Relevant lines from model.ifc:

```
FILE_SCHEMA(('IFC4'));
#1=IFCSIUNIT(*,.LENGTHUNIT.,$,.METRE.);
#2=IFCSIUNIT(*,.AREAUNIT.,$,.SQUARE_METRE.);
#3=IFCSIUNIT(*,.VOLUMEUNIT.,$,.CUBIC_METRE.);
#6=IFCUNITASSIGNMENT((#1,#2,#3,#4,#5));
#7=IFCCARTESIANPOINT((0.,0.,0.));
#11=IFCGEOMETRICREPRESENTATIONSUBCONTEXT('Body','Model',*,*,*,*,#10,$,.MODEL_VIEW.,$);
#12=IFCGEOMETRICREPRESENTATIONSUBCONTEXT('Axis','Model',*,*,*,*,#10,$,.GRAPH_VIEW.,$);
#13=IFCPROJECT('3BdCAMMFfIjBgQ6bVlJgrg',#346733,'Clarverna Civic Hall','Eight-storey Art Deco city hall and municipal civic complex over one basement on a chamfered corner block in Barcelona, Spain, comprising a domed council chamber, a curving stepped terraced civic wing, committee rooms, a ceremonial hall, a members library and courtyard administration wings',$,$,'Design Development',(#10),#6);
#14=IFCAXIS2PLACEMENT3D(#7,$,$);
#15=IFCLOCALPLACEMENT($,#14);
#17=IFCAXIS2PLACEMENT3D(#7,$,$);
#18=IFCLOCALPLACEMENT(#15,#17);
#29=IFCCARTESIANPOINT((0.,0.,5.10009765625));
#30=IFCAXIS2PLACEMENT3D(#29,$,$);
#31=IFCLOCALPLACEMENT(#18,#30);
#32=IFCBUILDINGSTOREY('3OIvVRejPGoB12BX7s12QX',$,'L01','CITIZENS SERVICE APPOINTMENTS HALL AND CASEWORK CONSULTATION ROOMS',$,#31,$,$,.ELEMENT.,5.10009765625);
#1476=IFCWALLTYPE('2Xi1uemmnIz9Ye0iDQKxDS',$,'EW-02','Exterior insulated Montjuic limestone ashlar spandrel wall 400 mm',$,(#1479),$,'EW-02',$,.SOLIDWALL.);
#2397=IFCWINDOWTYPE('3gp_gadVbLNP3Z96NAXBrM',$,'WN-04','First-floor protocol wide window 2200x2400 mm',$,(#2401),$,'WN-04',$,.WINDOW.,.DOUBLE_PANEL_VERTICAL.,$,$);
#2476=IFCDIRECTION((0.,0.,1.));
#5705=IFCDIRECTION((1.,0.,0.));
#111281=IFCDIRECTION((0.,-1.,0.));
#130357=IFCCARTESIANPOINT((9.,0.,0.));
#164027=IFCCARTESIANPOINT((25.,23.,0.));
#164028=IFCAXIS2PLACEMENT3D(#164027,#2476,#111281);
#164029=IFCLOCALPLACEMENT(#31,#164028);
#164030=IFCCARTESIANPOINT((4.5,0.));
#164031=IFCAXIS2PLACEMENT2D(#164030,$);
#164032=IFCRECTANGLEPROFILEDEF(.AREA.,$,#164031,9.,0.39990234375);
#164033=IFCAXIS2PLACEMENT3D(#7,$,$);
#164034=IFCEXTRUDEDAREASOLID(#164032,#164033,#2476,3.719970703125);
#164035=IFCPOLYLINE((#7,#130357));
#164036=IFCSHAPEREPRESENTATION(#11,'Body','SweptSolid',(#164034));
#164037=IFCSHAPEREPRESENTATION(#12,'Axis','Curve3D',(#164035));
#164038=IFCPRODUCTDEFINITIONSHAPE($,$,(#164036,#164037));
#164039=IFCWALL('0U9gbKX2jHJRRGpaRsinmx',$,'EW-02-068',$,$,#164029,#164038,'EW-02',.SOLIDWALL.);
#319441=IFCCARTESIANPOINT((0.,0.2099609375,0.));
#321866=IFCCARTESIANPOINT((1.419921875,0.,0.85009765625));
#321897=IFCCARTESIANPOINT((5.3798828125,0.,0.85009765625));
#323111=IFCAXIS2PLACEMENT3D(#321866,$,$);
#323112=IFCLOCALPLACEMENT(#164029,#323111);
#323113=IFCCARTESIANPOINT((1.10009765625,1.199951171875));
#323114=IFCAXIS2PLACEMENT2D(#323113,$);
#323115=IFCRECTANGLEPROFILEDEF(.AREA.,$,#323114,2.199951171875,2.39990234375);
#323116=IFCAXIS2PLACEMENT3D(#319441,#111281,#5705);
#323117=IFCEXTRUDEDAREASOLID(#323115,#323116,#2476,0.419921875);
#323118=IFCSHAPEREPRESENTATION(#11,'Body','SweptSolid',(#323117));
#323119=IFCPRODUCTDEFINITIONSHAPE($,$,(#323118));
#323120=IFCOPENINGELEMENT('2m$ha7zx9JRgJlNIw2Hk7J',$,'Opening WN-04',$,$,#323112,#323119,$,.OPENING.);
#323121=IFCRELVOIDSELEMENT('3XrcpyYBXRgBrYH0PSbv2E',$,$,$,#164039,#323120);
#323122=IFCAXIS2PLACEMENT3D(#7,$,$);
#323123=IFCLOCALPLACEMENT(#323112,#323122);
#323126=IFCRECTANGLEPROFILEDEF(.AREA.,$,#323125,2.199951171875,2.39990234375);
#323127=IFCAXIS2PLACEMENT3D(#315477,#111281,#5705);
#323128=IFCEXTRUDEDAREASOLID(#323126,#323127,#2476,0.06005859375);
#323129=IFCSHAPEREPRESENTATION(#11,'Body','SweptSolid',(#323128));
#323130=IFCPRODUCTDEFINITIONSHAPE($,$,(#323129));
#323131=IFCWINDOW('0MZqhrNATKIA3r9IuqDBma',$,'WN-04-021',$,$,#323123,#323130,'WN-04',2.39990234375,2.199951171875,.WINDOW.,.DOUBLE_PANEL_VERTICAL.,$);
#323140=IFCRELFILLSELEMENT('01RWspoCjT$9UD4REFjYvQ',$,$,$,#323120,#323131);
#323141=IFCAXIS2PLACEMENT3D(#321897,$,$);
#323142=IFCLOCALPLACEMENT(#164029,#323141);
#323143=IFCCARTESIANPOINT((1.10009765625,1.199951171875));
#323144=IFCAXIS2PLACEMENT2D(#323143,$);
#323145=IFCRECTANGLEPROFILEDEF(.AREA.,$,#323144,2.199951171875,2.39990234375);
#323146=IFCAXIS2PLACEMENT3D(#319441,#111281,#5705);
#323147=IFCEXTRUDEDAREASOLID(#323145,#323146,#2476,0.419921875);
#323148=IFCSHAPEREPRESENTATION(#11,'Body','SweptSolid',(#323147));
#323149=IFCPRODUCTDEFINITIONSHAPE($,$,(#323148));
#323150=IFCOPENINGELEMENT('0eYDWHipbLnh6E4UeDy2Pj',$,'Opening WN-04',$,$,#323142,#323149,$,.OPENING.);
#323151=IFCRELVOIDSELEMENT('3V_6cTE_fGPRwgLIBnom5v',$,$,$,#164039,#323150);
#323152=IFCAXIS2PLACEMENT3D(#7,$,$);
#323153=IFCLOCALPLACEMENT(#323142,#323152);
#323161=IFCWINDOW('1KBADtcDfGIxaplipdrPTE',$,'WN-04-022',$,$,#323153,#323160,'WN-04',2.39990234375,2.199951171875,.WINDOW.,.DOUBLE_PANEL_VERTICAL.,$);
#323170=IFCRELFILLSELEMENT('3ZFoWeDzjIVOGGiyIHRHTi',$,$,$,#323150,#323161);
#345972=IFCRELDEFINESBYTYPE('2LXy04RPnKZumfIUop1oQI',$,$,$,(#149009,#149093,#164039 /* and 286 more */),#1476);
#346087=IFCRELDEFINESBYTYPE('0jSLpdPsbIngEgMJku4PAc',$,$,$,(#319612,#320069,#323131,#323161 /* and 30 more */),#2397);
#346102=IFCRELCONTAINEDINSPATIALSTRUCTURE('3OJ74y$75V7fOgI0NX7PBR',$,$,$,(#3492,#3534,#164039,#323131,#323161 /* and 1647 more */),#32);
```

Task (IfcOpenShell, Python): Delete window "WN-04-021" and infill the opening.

```python
import ifcopenshell
import ifcopenshell.api.feature
import ifcopenshell.api.root
import ifcopenshell.geom
import ifcopenshell.util.shape

model = ifcopenshell.open("model.ifc")
settings = ifcopenshell.geom.settings()


def volume(element):
    """Net volume in cubic metres, openings subtracted."""
    shape = ifcopenshell.geom.create_shape(settings, element)
    return ifcopenshell.util.shape.get_volume(shape.geometry)


window = model.by_guid("0MZqhrNATKIA3r9IuqDBma")
opening = window.FillsVoids[0].RelatingOpeningElement
wall = opening.VoidsElements[0].RelatingBuildingElement
before = volume(wall)

ifcopenshell.api.root.remove_product(model, product=window)
ifcopenshell.api.feature.remove_feature(model, feature=opening)

after = volume(wall)

print(f"wall volume {before:.3f} -> {after:.3f} m3")

model.write("model_v2.ifc")
```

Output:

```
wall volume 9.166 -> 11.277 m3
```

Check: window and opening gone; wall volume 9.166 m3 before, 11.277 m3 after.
